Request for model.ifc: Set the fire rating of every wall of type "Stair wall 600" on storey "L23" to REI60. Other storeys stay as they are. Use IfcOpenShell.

First a look at what the model holds.

```python
import ifcopenshell
import ifcopenshell.util.element

model = ifcopenshell.open("model.ifc")
print(model.schema)
storey = next(s for s in model.by_type("IfcBuildingStorey") if s.Name == "L23")
walls = [e for e in ifcopenshell.util.element.get_decomposition(storey) if e.is_a("IfcWall")]
seen = {}
for e in walls:
    element_type = ifcopenshell.util.element.get_type(e)
    key = (element_type.Name if element_type != e and element_type else None, ifcopenshell.util.element.get_pset(e, "Pset_WallCommon", "FireRating"))
    seen[key] = seen.get(key, 0) + 1
for (name, value), count in sorted(seen.items(), key=str):
    print(count, "x", name, "|", value)
```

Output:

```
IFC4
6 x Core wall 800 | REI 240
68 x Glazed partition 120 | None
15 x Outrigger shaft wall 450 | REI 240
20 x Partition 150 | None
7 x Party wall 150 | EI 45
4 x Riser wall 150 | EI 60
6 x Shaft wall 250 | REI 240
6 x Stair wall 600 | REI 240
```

```python
import ifcopenshell
import ifcopenshell.api.pset
import ifcopenshell.util.element

model = ifcopenshell.open("model.ifc")

storey = next(s for s in model.by_type("IfcBuildingStorey") if s.Name == "L23")
walls = [e for e in ifcopenshell.util.element.get_decomposition(storey) if e.is_a("IfcWall")]

count = 0
for e in walls:
    element_type = ifcopenshell.util.element.get_type(e)
    if element_type in (None, e) or element_type.Name != "Stair wall 600":
        continue
    found = ifcopenshell.util.element.get_pset(e, "Pset_WallCommon", should_inherit=False)
    if found:
        pset = model.by_id(found["id"])
        if len(ifcopenshell.util.element.get_elements_by_pset(pset)) > 1:
            pset = ifcopenshell.api.pset.unshare_pset(model, products=[e], pset=pset)[0]
    else:
        pset = ifcopenshell.api.pset.add_pset(model, product=e, name="Pset_WallCommon")
    ifcopenshell.api.pset.edit_pset(model, pset=pset, properties={"FireRating": "REI60"})
    count += 1

print(count, "walls updated")

model.write("model_updated.ifc")
```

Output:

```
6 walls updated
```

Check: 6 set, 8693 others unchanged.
